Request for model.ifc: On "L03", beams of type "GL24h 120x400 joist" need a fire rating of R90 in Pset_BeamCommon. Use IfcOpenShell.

First a look at what the model holds.

```python
import ifcopenshell
import ifcopenshell.util.element

model = ifcopenshell.open("model.ifc")
print(model.schema)
storey = next(s for s in model.by_type("IfcBuildingStorey") if s.Name == "L03")
beams = [e for e in ifcopenshell.util.element.get_decomposition(storey) if e.is_a("IfcBeam")]
seen = {}
for e in beams:
    element_type = ifcopenshell.util.element.get_type(e)
    key = (element_type.Name if element_type != e and element_type else None, ifcopenshell.util.element.get_pset(e, "Pset_BeamCommon", "FireRating"))
    seen[key] = seen.get(key, 0) + 1
for (name, value), count in sorted(seen.items(), key=str):
    print(count, "x", name, "|", value)
```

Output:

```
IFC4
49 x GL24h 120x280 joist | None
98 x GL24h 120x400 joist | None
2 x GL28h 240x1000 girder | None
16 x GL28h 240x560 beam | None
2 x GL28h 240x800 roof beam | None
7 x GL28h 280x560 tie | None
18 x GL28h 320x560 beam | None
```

```python
import ifcopenshell
import ifcopenshell.api.pset
import ifcopenshell.util.element

model = ifcopenshell.open("model.ifc")

storey = next(s for s in model.by_type("IfcBuildingStorey") if s.Name == "L03")
beams = [e for e in ifcopenshell.util.element.get_decomposition(storey) if e.is_a("IfcBeam")]

count = 0
for e in beams:
    element_type = ifcopenshell.util.element.get_type(e)
    if element_type in (None, e) or element_type.Name != "GL24h 120x400 joist":
        continue
    # add_pset returns the element's existing set when there is one.
    pset = ifcopenshell.api.pset.add_pset(model, product=e, name="Pset_BeamCommon")
    ifcopenshell.api.pset.edit_pset(model, pset=pset, properties={"FireRating": "R90"})
    count += 1

print(count, "beams updated")

model.write("model-out.ifc")
```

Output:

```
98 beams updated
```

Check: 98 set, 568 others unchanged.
